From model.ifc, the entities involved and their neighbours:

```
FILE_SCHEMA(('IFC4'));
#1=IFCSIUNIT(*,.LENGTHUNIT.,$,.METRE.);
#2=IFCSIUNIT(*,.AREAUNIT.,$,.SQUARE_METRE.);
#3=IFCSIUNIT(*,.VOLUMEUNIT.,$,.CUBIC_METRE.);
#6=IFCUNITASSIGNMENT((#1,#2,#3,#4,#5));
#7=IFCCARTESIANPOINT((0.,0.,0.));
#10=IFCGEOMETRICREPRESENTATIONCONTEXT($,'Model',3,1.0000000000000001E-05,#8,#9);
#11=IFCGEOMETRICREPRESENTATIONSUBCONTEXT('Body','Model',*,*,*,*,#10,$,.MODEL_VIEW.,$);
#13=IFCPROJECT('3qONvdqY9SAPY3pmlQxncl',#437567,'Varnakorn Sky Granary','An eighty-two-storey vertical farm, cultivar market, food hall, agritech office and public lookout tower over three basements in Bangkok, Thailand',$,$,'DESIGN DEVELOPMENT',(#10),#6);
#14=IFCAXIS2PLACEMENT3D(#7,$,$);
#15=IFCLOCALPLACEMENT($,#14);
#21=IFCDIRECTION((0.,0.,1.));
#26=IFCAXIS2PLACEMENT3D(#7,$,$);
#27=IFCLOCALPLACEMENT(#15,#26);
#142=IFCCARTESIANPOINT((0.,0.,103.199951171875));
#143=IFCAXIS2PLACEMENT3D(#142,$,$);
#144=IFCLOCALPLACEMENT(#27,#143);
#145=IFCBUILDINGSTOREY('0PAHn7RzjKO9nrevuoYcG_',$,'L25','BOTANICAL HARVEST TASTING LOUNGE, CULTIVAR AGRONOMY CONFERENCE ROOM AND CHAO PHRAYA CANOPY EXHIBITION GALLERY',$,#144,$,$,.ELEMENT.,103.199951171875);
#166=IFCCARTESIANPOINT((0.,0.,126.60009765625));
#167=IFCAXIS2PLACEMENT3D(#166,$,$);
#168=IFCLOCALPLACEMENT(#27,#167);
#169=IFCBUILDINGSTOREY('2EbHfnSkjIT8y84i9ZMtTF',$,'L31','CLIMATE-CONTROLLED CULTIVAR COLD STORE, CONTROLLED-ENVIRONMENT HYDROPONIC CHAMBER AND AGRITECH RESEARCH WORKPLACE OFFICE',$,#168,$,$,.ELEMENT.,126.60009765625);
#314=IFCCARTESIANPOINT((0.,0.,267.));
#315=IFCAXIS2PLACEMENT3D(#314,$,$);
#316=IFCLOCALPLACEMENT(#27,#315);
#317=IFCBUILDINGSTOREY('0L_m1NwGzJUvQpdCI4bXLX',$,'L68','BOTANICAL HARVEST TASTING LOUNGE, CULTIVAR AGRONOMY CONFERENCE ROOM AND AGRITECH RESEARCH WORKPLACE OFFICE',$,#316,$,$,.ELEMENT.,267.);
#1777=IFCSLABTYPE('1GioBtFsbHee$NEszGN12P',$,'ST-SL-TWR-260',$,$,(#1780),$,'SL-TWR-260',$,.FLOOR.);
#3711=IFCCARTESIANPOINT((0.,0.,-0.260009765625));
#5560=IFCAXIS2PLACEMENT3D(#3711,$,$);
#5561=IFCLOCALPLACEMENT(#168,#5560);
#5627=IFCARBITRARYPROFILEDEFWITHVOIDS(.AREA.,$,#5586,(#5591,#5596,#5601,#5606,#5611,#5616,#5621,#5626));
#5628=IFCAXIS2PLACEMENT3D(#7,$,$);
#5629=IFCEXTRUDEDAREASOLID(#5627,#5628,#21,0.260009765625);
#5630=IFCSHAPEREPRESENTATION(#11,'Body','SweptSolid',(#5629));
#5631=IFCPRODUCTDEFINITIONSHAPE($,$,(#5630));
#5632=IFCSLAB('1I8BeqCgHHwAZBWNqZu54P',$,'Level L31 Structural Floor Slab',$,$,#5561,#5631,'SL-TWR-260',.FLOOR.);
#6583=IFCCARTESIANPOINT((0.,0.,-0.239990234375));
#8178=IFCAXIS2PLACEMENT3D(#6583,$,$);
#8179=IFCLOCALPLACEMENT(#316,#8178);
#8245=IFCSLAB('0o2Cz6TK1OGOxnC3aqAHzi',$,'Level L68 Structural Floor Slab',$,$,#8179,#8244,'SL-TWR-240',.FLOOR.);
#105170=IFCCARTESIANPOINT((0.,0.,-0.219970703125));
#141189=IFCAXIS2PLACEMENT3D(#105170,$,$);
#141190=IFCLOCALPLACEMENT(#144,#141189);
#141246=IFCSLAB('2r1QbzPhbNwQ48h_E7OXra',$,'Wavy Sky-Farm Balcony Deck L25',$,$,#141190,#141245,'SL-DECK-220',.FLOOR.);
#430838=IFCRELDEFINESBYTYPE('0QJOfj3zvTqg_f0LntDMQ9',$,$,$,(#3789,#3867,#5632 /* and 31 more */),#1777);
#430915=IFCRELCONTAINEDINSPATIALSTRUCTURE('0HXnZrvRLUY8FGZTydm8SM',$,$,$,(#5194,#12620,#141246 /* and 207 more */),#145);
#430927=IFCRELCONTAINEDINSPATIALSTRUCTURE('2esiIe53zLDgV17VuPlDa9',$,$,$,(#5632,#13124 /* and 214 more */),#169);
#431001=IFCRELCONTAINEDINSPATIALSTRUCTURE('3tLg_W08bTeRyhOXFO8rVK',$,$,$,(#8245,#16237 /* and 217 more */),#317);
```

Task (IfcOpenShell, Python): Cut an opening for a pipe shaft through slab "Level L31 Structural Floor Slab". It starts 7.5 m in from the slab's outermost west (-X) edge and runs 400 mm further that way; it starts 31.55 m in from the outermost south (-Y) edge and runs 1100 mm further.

```python
import numpy as np
import ifcopenshell
import ifcopenshell.api.feature
import ifcopenshell.api.geometry
import ifcopenshell.api.root
import ifcopenshell.geom
import ifcopenshell.util.placement
import ifcopenshell.util.representation
import ifcopenshell.util.shape
import ifcopenshell.util.unit

model = ifcopenshell.open("model.ifc")
unit_scale = ifcopenshell.util.unit.calculate_unit_scale(model)
settings = ifcopenshell.geom.settings()


def volume(element):
    """Net volume in cubic metres, openings subtracted."""
    shape = ifcopenshell.geom.create_shape(settings, element)
    return ifcopenshell.util.shape.get_volume(shape.geometry)


slab = model.by_guid("1I8BeqCgHHwAZBWNqZu54P")
before = volume(slab)

# Extent in the slab's own axes, in metres. The edges named are its -X and -Y sides.
slab_shape = ifcopenshell.geom.create_shape(settings, slab)
vertices = ifcopenshell.util.shape.get_vertices(slab_shape.geometry)
x_min, y_min, bottom = vertices.min(axis=0)
top = vertices[:, 2].max()

opening = ifcopenshell.api.root.create_entity(model, ifc_class="IfcOpeningElement", name="Pipe shaft opening", predefined_type="OPENING")
context = ifcopenshell.util.representation.get_context(model, "Model", "Body", "MODEL_VIEW")
width, depth = 0.4, 1.1
outline = [(0.0, 0.0), (width, 0.0), (width, depth), (0.0, depth), (0.0, 0.0)]
# Overshoot both faces by 50 mm so the cut is clean.
shape = ifcopenshell.api.geometry.add_slab_representation(
    model, context=context, depth=top - bottom + 0.1, polyline=outline
)
ifcopenshell.api.geometry.assign_representation(model, product=opening, representation=shape)

matrix = ifcopenshell.util.placement.get_local_placement(slab.ObjectPlacement)
matrix[:, 3] = matrix @ np.append(np.array([x_min + 7.5, y_min + 31.55, bottom - 0.05]) / unit_scale, 1.0)
ifcopenshell.api.geometry.edit_object_placement(model, product=opening, matrix=matrix, is_si=False)
ifcopenshell.api.feature.add_feature(model, feature=opening, element=slab)

after = volume(slab)

print(f"slab volume {before:.3f} -> {after:.3f} m3")

model.write("model_updated.ifc")
```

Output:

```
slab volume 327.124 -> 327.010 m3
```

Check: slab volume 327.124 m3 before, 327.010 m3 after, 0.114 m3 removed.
